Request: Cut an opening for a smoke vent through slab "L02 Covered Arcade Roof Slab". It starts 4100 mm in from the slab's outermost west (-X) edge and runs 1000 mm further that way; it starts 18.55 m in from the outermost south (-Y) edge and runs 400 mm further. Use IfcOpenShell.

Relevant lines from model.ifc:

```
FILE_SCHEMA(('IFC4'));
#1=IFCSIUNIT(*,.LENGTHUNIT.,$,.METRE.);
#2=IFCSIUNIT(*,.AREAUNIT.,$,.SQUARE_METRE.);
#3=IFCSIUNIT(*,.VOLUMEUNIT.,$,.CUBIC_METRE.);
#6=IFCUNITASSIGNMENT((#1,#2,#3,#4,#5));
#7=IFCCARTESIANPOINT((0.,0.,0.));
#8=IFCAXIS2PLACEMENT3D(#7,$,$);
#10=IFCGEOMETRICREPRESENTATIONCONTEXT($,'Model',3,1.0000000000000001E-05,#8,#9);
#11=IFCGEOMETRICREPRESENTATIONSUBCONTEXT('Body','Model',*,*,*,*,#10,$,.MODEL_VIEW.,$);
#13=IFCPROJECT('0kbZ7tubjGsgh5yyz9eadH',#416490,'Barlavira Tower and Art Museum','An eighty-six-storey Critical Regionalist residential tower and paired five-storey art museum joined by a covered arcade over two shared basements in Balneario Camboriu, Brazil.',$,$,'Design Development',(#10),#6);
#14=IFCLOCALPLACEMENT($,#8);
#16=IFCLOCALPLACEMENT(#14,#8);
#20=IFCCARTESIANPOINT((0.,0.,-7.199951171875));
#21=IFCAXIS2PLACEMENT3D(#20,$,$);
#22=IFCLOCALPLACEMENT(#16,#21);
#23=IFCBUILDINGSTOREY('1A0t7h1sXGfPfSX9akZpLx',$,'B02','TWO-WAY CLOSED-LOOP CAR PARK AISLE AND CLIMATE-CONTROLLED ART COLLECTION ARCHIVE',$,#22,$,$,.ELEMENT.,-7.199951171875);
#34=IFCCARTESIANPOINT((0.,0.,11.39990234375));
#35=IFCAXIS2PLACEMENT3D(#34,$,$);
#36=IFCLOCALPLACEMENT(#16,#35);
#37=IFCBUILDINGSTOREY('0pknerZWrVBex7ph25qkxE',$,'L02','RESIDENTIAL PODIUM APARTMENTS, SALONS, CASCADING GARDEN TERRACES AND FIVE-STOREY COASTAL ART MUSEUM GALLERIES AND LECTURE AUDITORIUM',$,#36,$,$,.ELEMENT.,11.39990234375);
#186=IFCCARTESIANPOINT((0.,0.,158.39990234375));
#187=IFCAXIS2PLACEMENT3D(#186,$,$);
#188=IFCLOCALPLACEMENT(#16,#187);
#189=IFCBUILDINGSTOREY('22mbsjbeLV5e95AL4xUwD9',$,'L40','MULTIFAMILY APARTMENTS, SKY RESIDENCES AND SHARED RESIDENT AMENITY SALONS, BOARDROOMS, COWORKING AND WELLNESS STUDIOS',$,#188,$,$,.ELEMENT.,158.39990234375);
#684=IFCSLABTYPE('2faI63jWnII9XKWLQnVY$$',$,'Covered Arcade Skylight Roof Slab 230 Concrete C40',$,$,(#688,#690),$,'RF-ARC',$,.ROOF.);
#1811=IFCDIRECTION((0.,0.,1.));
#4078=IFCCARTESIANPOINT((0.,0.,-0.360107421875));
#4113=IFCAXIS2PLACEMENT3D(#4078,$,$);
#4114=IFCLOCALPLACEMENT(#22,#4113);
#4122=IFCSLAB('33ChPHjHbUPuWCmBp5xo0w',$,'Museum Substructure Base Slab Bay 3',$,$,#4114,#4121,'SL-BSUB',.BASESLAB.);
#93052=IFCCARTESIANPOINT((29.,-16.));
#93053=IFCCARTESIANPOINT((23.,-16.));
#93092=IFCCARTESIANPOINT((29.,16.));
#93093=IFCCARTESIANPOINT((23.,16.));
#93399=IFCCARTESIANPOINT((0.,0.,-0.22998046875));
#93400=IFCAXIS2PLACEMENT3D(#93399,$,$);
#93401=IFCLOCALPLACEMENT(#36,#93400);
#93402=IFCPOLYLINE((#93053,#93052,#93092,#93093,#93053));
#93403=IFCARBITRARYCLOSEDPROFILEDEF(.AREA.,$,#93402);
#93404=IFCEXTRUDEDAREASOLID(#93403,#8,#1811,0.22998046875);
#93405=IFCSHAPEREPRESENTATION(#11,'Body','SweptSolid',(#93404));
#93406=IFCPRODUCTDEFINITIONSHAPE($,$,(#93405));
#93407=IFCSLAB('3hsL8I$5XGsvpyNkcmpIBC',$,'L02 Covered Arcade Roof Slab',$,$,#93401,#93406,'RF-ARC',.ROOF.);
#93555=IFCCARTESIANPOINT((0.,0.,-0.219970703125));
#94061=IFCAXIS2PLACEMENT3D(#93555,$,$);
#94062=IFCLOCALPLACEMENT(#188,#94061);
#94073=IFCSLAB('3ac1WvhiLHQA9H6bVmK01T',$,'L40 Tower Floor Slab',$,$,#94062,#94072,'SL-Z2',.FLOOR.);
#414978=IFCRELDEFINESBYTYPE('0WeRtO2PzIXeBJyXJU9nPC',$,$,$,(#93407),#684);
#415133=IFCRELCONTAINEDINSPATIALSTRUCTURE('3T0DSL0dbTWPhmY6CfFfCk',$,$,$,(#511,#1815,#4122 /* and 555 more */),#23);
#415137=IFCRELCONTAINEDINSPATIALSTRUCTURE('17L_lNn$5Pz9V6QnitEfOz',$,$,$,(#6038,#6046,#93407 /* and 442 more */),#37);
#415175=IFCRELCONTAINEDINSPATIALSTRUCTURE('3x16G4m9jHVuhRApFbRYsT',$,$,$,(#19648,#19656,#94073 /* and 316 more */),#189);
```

```python
import numpy as np
import ifcopenshell
import ifcopenshell.api.feature
import ifcopenshell.api.geometry
import ifcopenshell.api.root
import ifcopenshell.geom
import ifcopenshell.util.placement
import ifcopenshell.util.representation
import ifcopenshell.util.shape
import ifcopenshell.util.unit

model = ifcopenshell.open("model.ifc")
unit_scale = ifcopenshell.util.unit.calculate_unit_scale(model)
settings = ifcopenshell.geom.settings()


def volume(element):
    """Net volume in cubic metres, openings subtracted."""
    shape = ifcopenshell.geom.create_shape(settings, element)
    return ifcopenshell.util.shape.get_volume(shape.geometry)


slab = model.by_guid("3hsL8I$5XGsvpyNkcmpIBC")
before = volume(slab)

# Extent in the slab's own axes, in metres. The edges named are its -X and -Y sides.
slab_shape = ifcopenshell.geom.create_shape(settings, slab)
vertices = ifcopenshell.util.shape.get_vertices(slab_shape.geometry)
x_min, y_min, bottom = vertices.min(axis=0)
top = vertices[:, 2].max()

opening = ifcopenshell.api.root.create_entity(model, ifc_class="IfcOpeningElement", name="Smoke vent opening", predefined_type="OPENING")
context = ifcopenshell.util.representation.get_context(model, "Model", "Body", "MODEL_VIEW")
width, depth = 1, 0.4
outline = [(0.0, 0.0), (width, 0.0), (width, depth), (0.0, depth), (0.0, 0.0)]
# Overshoot both faces by 50 mm so the cut is clean.
shape = ifcopenshell.api.geometry.add_slab_representation(
    model, context=context, depth=top - bottom + 0.1, polyline=outline
)
ifcopenshell.api.geometry.assign_representation(model, product=opening, representation=shape)

matrix = ifcopenshell.util.placement.get_local_placement(slab.ObjectPlacement)
matrix[:, 3] = matrix @ np.append(np.array([x_min + 4.1, y_min + 18.55, bottom - 0.05]) / unit_scale, 1.0)
ifcopenshell.api.geometry.edit_object_placement(model, product=opening, matrix=matrix, is_si=False)
ifcopenshell.api.feature.add_feature(model, feature=opening, element=slab)

after = volume(slab)

print(f"slab volume {before:.3f} -> {after:.3f} m3")

model.write("model_v2.ifc")
```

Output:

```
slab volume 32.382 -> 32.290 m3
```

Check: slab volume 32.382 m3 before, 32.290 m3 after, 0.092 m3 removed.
